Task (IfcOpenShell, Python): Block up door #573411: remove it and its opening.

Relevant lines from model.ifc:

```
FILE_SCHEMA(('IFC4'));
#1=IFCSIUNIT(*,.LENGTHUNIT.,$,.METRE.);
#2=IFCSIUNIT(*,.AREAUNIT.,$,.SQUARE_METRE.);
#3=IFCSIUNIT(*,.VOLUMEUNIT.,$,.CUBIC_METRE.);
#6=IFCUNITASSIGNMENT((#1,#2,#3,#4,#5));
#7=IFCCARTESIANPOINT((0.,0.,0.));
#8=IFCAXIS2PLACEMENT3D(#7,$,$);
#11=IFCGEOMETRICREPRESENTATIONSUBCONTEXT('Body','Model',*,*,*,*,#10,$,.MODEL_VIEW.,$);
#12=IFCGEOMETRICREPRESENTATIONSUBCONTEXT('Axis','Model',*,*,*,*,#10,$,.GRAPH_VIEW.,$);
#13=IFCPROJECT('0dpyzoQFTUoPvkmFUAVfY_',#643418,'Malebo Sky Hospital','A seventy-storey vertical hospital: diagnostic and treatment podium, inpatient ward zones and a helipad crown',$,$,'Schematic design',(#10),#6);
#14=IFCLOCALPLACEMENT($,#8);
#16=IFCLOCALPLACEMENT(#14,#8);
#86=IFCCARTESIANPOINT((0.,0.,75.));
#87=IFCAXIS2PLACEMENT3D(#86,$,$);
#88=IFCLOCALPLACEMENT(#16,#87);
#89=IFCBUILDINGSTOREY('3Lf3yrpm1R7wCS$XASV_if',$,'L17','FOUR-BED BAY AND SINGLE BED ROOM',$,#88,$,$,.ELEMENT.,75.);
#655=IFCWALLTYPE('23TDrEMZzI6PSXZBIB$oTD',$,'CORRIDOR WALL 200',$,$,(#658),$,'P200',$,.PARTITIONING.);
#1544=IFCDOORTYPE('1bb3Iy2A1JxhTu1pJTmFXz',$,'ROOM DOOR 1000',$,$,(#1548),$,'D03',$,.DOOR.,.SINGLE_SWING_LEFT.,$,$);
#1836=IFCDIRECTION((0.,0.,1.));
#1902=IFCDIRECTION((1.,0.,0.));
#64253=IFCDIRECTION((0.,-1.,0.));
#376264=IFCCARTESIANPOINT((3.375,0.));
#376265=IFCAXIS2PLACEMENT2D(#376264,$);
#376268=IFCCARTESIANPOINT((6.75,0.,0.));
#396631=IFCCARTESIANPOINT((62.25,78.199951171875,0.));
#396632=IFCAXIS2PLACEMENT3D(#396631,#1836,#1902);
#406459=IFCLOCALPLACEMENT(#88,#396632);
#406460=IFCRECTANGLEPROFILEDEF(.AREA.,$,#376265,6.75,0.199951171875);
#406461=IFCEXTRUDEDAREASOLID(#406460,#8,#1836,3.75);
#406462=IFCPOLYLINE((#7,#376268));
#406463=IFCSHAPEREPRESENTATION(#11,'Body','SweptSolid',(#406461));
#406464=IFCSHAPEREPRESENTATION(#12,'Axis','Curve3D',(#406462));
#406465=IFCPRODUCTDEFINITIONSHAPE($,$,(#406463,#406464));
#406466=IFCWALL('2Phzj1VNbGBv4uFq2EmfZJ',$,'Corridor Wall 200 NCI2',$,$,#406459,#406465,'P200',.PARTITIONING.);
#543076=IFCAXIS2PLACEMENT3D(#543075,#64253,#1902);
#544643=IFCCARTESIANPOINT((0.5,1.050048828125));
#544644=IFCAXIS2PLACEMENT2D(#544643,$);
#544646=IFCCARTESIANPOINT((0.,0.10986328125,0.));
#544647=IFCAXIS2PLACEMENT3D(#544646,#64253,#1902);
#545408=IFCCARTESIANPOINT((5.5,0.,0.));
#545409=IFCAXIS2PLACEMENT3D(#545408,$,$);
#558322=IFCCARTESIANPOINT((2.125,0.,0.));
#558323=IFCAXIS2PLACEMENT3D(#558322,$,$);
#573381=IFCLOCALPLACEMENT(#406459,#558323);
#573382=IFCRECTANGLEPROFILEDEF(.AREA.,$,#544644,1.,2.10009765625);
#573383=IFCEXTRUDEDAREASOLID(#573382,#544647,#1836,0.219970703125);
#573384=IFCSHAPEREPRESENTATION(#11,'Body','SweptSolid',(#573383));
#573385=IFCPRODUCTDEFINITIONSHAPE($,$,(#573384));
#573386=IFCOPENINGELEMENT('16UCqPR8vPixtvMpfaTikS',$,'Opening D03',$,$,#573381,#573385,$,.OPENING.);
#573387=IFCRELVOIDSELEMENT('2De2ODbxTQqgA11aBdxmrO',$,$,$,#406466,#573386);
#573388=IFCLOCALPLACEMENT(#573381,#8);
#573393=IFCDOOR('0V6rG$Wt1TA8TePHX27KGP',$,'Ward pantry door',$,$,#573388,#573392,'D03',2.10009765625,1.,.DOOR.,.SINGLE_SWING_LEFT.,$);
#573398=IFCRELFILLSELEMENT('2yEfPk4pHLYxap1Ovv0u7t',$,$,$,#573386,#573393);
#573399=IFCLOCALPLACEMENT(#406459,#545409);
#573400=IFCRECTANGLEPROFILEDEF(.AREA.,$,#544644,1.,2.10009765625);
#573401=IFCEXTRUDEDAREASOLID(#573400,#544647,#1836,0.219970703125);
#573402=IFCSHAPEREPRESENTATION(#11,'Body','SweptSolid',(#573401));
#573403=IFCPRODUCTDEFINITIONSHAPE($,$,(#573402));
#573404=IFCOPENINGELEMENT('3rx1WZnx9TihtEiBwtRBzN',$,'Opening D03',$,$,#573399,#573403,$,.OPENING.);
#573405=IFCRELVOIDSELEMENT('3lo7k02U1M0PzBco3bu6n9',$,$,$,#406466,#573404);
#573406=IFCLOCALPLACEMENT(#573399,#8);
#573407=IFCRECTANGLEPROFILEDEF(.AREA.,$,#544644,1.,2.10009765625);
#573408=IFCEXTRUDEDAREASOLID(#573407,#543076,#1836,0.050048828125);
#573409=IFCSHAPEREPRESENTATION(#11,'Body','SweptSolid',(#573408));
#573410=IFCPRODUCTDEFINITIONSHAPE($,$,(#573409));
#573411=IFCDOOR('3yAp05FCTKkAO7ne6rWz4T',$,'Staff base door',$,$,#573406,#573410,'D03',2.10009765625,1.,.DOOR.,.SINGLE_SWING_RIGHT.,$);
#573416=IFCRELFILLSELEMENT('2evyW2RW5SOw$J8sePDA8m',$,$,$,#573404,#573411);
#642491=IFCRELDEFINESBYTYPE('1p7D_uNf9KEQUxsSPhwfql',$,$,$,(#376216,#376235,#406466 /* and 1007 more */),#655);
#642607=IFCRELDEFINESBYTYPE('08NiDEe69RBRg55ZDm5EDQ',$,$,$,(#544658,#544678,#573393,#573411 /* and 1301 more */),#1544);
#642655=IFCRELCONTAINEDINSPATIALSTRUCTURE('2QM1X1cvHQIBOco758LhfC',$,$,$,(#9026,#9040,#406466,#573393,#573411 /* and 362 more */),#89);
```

```python
import ifcopenshell
import ifcopenshell.api.feature
import ifcopenshell.api.root
import ifcopenshell.geom
import ifcopenshell.util.shape

model = ifcopenshell.open("model.ifc")
settings = ifcopenshell.geom.settings()


def volume(element):
    """Net volume in cubic metres, openings subtracted."""
    shape = ifcopenshell.geom.create_shape(settings, element)
    return ifcopenshell.util.shape.get_volume(shape.geometry)


door = model.by_id(573411)
opening = door.FillsVoids[0].RelatingOpeningElement
wall = opening.VoidsElements[0].RelatingBuildingElement
before = volume(wall)

ifcopenshell.api.root.remove_product(model, product=door)
ifcopenshell.api.feature.remove_feature(model, feature=opening)

after = volume(wall)

print(f"wall volume {before:.3f} -> {after:.3f} m3")

model.write("model_edited.ifc")
```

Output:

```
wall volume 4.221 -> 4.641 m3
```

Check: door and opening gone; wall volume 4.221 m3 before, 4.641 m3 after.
